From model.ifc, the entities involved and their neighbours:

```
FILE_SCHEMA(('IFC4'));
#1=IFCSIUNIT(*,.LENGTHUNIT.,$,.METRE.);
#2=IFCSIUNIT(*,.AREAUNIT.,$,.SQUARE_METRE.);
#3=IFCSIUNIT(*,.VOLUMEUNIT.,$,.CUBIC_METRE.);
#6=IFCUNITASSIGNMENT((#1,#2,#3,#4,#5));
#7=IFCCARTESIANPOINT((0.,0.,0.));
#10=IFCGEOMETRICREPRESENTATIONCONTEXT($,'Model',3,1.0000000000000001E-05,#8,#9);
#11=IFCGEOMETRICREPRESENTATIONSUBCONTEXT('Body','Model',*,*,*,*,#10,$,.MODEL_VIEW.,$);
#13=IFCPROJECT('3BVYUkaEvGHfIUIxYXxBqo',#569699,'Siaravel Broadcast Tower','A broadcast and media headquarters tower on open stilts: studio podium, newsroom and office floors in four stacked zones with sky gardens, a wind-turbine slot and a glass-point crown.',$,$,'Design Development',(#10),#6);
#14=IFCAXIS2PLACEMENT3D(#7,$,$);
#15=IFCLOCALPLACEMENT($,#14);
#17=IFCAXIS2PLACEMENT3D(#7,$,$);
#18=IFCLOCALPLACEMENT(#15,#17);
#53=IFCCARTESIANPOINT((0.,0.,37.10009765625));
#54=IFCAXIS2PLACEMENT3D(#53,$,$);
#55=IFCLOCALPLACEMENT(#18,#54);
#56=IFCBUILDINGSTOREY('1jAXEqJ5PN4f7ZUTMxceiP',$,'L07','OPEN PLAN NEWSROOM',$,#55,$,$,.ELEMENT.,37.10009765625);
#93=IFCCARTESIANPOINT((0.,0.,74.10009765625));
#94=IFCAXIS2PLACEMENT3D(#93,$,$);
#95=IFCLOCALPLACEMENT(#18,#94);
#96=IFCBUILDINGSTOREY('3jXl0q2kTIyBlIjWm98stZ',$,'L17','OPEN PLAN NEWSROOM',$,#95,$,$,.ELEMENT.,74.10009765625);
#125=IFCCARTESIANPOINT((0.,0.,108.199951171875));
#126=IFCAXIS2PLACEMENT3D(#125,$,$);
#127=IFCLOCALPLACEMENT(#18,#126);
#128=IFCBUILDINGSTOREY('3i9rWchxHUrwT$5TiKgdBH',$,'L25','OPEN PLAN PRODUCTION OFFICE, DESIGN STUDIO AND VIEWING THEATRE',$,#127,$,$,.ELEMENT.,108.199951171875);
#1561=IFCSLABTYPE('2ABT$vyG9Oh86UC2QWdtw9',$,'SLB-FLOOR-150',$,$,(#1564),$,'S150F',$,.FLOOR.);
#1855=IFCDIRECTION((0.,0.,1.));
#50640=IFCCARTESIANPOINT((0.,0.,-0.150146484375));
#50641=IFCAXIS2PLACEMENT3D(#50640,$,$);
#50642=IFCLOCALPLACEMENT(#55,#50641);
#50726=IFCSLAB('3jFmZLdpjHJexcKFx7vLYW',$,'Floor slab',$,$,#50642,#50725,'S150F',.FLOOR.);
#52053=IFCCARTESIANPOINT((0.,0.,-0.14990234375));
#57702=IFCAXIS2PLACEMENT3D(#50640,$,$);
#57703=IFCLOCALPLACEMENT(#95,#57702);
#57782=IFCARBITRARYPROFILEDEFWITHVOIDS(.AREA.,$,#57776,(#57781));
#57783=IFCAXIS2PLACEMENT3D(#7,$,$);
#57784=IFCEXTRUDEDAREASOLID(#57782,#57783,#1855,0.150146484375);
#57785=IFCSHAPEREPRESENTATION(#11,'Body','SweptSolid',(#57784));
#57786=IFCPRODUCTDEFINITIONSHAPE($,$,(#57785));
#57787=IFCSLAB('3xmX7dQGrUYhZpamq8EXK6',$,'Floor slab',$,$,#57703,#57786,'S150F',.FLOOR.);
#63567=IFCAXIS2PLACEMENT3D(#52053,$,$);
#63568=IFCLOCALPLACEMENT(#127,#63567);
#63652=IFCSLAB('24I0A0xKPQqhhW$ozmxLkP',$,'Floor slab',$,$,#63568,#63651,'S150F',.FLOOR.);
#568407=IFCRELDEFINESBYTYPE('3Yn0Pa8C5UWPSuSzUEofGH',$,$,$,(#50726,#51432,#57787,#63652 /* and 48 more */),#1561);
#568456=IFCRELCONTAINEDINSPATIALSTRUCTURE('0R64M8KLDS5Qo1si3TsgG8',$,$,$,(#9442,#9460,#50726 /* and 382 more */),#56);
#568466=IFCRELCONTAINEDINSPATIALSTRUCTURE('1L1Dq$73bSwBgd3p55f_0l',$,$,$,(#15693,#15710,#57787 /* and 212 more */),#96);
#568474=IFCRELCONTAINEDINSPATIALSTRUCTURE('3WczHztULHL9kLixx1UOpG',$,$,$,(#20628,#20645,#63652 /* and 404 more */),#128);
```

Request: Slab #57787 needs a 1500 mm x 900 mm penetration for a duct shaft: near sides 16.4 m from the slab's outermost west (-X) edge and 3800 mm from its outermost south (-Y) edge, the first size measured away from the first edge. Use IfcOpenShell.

```python
import numpy as np
import ifcopenshell
import ifcopenshell.api.feature
import ifcopenshell.api.geometry
import ifcopenshell.api.root
import ifcopenshell.geom
import ifcopenshell.util.placement
import ifcopenshell.util.representation
import ifcopenshell.util.shape
import ifcopenshell.util.unit

model = ifcopenshell.open("model.ifc")
unit_scale = ifcopenshell.util.unit.calculate_unit_scale(model)
settings = ifcopenshell.geom.settings()


def volume(element):
    """Net volume in cubic metres, openings subtracted."""
    shape = ifcopenshell.geom.create_shape(settings, element)
    return ifcopenshell.util.shape.get_volume(shape.geometry)


slab = model.by_id(57787)
before = volume(slab)

# Extent in the slab's own axes, in metres. The edges named are its -X and -Y sides.
slab_shape = ifcopenshell.geom.create_shape(settings, slab)
vertices = ifcopenshell.util.shape.get_vertices(slab_shape.geometry)
x_min, y_min, bottom = vertices.min(axis=0)
top = vertices[:, 2].max()

opening = ifcopenshell.api.root.create_entity(model, ifc_class="IfcOpeningElement", name="Duct shaft opening", predefined_type="OPENING")
context = ifcopenshell.util.representation.get_context(model, "Model", "Body", "MODEL_VIEW")
width, depth = 1.5, 0.9
outline = [(0.0, 0.0), (width, 0.0), (width, depth), (0.0, depth), (0.0, 0.0)]
# Overshoot both faces by 50 mm so the cut is clean.
shape = ifcopenshell.api.geometry.add_slab_representation(
    model, context=context, depth=top - bottom + 0.1, polyline=outline
)
ifcopenshell.api.geometry.assign_representation(model, product=opening, representation=shape)

matrix = ifcopenshell.util.placement.get_local_placement(slab.ObjectPlacement)
matrix[:, 3] = matrix @ np.append(np.array([x_min + 16.4, y_min + 3.8, bottom - 0.05]) / unit_scale, 1.0)
ifcopenshell.api.geometry.edit_object_placement(model, product=opening, matrix=matrix, is_si=False)
ifcopenshell.api.feature.add_feature(model, feature=opening, element=slab)

after = volume(slab)

print(f"slab volume {before:.3f} -> {after:.3f} m3")

model.write("model_rev.ifc")
```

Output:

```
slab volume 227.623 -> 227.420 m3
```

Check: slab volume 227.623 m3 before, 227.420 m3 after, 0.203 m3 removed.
